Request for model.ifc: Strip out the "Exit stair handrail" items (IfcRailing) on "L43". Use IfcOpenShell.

First a look at what the model holds.

```python
import ifcopenshell
import ifcopenshell.util.element

model = ifcopenshell.open("model.ifc")
print(model.schema)
storey = next(s for s in model.by_type("IfcBuildingStorey") if s.Name == "L43")
railings = [e for e in ifcopenshell.util.element.get_decomposition(storey) if e.is_a("IfcRailing")]
seen = {}
for e in railings:
    element_type = ifcopenshell.util.element.get_type(e)
    name = element_type.Name if element_type not in (None, e) else None
    seen[name] = seen.get(name, 0) + 1
for name, count in sorted(seen.items(), key=str):
    print(count, "x", name)
```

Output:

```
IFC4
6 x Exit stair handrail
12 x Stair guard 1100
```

```python
import ifcopenshell
import ifcopenshell.api.root
import ifcopenshell.util.element

model = ifcopenshell.open("model.ifc")

storey = next(s for s in model.by_type("IfcBuildingStorey") if s.Name == "L43")
railings = [e for e in ifcopenshell.util.element.get_decomposition(storey) if e.is_a("IfcRailing")]
targets = [e for e in railings if (t := ifcopenshell.util.element.get_type(e)) not in (None, e) and t.Name == "Exit stair handrail"]

for e in targets:
    ifcopenshell.api.root.remove_product(model, product=e)
print(len(targets), "removed")

model.write("model-out.ifc")
```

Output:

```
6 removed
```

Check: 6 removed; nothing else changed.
